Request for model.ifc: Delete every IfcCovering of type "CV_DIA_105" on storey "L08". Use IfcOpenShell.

First a look at what the model holds.

```python
import ifcopenshell
import ifcopenshell.util.element

model = ifcopenshell.open("model.ifc")
print(model.schema)
storey = next(s for s in model.by_type("IfcBuildingStorey") if s.Name == "L08")
coverings = [e for e in ifcopenshell.util.element.get_decomposition(storey) if e.is_a("IfcCovering")]
seen = {}
for e in coverings:
    element_type = ifcopenshell.util.element.get_type(e)
    name = element_type.Name if element_type not in (None, e) else None
    seen[name] = seen.get(name, 0) + 1
for name, count in sorted(seen.items(), key=str):
    print(count, "x", name)
```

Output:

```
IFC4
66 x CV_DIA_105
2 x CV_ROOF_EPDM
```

```python
import ifcopenshell
import ifcopenshell.api.root
import ifcopenshell.util.element

model = ifcopenshell.open("model.ifc")

storey = next(s for s in model.by_type("IfcBuildingStorey") if s.Name == "L08")
coverings = [e for e in ifcopenshell.util.element.get_decomposition(storey) if e.is_a("IfcCovering")]
targets = [e for e in coverings if (t := ifcopenshell.util.element.get_type(e)) not in (None, e) and t.Name == "CV_DIA_105"]

for e in targets:
    ifcopenshell.api.root.remove_product(model, product=e)
print(len(targets), "removed")

model.write("model-out.ifc")
```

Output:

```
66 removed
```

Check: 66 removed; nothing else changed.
